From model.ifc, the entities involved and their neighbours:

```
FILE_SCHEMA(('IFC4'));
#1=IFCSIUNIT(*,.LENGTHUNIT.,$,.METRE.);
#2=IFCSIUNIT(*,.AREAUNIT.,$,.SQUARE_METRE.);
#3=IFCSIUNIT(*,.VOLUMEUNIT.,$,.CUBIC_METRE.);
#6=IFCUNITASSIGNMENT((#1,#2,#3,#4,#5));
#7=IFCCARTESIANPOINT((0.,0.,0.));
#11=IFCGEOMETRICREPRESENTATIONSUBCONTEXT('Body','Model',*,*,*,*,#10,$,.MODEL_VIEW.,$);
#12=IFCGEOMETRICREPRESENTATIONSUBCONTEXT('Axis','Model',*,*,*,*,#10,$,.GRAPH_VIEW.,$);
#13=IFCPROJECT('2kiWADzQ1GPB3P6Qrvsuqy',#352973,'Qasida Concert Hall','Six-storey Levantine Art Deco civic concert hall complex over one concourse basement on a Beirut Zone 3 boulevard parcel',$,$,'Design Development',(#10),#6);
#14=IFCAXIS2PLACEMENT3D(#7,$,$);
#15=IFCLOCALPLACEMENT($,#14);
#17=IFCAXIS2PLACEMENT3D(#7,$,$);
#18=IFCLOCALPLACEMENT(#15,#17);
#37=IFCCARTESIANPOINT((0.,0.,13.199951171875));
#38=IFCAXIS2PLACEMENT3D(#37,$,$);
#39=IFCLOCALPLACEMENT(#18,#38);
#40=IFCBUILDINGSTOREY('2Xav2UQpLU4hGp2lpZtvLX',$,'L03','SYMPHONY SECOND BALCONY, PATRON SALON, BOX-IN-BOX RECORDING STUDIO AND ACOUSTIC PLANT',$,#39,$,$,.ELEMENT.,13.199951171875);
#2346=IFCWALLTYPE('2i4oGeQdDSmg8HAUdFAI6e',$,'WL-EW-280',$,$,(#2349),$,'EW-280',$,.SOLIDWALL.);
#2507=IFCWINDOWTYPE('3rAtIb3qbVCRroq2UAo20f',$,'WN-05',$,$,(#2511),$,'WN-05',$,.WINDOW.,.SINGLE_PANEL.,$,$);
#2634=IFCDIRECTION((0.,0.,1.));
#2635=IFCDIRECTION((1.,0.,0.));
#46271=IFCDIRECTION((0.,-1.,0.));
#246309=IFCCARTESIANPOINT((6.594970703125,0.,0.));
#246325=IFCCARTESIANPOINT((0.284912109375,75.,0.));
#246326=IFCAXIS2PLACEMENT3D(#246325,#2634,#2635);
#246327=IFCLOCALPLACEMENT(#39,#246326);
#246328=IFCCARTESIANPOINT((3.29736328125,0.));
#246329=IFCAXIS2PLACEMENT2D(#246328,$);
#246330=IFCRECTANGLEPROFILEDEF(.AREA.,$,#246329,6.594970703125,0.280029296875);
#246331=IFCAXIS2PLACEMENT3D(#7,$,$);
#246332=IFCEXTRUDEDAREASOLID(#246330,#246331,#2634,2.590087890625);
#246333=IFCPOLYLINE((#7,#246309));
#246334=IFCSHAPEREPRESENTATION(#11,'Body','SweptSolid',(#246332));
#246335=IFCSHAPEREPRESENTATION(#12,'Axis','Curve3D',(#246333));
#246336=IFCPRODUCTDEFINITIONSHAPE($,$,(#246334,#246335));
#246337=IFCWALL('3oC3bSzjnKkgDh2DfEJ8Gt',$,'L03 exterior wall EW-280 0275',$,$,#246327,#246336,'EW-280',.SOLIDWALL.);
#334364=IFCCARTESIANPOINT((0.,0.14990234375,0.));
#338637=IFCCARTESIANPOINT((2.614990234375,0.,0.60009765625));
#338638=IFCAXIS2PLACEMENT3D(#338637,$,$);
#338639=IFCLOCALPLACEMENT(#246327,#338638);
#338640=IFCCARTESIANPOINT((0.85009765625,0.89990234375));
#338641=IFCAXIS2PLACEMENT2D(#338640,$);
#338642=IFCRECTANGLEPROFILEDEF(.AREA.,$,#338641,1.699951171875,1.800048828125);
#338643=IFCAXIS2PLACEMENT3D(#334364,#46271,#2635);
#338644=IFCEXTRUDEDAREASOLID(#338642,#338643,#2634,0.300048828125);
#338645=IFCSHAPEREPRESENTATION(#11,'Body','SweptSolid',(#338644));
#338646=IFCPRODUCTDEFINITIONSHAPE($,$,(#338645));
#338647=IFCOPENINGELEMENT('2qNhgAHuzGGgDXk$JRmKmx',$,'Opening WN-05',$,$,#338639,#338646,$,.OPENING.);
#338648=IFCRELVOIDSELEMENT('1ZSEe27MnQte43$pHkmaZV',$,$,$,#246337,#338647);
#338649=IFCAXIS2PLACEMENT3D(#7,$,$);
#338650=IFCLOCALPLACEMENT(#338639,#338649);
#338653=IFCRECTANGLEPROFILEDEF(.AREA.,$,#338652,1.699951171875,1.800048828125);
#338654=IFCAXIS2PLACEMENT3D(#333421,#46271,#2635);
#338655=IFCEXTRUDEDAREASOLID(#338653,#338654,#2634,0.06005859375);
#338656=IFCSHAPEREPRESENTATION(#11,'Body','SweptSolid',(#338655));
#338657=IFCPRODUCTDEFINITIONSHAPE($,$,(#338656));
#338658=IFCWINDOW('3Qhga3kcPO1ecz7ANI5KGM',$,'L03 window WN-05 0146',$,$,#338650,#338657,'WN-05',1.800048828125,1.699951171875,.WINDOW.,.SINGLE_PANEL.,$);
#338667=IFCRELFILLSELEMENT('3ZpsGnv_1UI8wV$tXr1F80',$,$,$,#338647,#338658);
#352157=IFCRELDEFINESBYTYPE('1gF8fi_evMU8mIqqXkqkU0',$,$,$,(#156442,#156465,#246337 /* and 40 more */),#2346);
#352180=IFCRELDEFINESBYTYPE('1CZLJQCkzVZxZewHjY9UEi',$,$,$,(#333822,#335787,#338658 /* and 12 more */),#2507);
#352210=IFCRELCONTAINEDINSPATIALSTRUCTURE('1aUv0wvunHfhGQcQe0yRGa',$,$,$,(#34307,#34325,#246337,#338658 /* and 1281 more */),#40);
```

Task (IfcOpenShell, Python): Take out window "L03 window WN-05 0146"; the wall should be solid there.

```python
import ifcopenshell
import ifcopenshell.api.feature
import ifcopenshell.api.root
import ifcopenshell.geom
import ifcopenshell.util.shape

model = ifcopenshell.open("model.ifc")
settings = ifcopenshell.geom.settings()


def volume(element):
    """Net volume in cubic metres, openings subtracted."""
    shape = ifcopenshell.geom.create_shape(settings, element)
    return ifcopenshell.util.shape.get_volume(shape.geometry)


window = model.by_guid("3Qhga3kcPO1ecz7ANI5KGM")
opening = window.FillsVoids[0].RelatingOpeningElement
wall = opening.VoidsElements[0].RelatingBuildingElement
before = volume(wall)

ifcopenshell.api.root.remove_product(model, product=window)
ifcopenshell.api.feature.remove_feature(model, feature=opening)

after = volume(wall)

print(f"wall volume {before:.3f} -> {after:.3f} m3")

model.write("model_edited.ifc")
```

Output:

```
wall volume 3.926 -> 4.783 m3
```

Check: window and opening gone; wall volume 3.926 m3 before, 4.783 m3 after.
